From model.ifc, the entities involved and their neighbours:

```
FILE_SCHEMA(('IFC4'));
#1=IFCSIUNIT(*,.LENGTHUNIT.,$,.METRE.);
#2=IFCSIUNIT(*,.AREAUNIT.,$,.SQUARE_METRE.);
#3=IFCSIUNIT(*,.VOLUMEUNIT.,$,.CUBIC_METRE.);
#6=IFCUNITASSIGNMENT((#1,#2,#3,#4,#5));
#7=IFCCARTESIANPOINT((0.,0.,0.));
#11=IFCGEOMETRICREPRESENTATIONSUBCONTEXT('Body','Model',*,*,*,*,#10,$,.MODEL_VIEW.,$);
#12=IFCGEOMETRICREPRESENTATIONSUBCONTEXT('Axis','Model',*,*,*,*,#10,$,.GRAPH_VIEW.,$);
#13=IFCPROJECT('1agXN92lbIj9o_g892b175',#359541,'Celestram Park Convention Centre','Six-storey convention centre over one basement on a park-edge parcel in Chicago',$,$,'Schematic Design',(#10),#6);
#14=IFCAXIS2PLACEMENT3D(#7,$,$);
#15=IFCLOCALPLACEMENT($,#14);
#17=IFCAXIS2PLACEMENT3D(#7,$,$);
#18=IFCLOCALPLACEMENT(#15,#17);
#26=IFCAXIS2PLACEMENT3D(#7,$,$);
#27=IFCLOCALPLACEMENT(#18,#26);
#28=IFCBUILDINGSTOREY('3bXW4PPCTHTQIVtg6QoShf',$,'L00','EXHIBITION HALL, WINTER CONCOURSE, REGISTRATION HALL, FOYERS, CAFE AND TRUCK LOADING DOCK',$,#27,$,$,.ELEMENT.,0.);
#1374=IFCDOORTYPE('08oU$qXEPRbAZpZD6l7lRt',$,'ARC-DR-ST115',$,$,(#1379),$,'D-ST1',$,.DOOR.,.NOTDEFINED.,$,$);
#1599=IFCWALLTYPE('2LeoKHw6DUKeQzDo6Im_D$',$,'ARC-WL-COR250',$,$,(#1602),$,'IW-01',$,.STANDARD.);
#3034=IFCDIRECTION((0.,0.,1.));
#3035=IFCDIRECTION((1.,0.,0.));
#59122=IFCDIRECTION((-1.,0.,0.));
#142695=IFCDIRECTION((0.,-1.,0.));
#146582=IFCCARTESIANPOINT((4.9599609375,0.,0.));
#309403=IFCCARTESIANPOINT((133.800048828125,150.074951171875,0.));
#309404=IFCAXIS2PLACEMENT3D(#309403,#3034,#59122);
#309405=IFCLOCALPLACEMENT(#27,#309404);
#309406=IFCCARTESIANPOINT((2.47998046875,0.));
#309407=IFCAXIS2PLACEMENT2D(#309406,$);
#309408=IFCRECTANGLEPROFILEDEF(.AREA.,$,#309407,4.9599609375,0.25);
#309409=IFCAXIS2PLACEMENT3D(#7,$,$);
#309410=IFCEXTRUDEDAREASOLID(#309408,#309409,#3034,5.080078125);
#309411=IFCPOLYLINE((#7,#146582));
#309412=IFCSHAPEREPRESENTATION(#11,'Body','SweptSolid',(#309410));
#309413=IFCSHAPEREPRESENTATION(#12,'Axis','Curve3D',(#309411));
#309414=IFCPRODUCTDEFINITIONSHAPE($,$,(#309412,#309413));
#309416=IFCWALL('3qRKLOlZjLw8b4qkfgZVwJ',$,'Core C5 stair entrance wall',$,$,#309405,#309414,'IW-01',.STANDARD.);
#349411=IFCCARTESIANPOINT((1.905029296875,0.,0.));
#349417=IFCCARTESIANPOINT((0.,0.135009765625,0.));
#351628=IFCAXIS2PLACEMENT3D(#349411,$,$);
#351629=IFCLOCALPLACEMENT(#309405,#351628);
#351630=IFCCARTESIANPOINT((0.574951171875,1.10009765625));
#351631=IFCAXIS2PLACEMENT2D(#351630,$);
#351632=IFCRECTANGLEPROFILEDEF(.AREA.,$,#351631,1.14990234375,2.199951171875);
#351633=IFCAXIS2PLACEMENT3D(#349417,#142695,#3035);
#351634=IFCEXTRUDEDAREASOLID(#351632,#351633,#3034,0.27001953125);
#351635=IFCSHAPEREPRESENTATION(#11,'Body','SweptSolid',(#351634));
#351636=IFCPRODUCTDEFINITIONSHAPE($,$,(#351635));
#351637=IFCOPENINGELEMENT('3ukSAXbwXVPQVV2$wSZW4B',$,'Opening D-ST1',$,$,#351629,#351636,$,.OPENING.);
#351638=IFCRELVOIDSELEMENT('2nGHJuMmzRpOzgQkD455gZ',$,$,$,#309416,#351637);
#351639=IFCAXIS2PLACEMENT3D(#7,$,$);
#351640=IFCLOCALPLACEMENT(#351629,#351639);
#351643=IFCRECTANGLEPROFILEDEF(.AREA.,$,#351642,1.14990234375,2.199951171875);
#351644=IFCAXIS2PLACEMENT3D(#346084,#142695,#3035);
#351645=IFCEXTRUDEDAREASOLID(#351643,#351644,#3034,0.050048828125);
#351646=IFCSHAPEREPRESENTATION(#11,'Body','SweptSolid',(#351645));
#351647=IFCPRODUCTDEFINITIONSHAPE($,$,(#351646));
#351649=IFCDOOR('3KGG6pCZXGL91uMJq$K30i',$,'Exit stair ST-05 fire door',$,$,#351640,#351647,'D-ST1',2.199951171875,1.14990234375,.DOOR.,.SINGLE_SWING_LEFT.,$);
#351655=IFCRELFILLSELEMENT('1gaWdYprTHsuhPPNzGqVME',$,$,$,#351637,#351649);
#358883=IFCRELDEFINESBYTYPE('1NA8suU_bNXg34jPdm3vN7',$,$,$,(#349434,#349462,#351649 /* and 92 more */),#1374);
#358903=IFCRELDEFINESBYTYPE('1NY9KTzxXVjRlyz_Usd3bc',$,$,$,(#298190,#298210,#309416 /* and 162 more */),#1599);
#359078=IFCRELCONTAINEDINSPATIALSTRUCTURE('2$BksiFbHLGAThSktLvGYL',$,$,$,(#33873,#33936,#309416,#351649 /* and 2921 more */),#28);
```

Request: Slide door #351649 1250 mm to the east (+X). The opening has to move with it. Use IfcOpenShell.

```python
import ifcopenshell
import ifcopenshell.api.geometry
import ifcopenshell.util.placement

model = ifcopenshell.open("model.ifc")

door = model.by_id(351649)
opening = door.FillsVoids[0].RelatingOpeningElement
wall = opening.VoidsElements[0].RelatingBuildingElement

wall_matrix = ifcopenshell.util.placement.get_local_placement(wall.ObjectPlacement)
shift = wall_matrix[:3, 0] * -1.25
before = ifcopenshell.util.placement.get_local_placement(door.ObjectPlacement)[:3, 3].copy()

# The door is placed relative to its opening, so it follows when the opening moves.
matrix = ifcopenshell.util.placement.get_local_placement(opening.ObjectPlacement)
matrix[:3, 3] += shift
ifcopenshell.api.geometry.edit_object_placement(
    model, product=opening, matrix=matrix, is_si=False, should_transform_children=True
)

after = ifcopenshell.util.placement.get_local_placement(door.ObjectPlacement)[:3, 3]
print("door moved by", (after - before).round(3) + 0.0)

model.write("model_rev.ifc")
```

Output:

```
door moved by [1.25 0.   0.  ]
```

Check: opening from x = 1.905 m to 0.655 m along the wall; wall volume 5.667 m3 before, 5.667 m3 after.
